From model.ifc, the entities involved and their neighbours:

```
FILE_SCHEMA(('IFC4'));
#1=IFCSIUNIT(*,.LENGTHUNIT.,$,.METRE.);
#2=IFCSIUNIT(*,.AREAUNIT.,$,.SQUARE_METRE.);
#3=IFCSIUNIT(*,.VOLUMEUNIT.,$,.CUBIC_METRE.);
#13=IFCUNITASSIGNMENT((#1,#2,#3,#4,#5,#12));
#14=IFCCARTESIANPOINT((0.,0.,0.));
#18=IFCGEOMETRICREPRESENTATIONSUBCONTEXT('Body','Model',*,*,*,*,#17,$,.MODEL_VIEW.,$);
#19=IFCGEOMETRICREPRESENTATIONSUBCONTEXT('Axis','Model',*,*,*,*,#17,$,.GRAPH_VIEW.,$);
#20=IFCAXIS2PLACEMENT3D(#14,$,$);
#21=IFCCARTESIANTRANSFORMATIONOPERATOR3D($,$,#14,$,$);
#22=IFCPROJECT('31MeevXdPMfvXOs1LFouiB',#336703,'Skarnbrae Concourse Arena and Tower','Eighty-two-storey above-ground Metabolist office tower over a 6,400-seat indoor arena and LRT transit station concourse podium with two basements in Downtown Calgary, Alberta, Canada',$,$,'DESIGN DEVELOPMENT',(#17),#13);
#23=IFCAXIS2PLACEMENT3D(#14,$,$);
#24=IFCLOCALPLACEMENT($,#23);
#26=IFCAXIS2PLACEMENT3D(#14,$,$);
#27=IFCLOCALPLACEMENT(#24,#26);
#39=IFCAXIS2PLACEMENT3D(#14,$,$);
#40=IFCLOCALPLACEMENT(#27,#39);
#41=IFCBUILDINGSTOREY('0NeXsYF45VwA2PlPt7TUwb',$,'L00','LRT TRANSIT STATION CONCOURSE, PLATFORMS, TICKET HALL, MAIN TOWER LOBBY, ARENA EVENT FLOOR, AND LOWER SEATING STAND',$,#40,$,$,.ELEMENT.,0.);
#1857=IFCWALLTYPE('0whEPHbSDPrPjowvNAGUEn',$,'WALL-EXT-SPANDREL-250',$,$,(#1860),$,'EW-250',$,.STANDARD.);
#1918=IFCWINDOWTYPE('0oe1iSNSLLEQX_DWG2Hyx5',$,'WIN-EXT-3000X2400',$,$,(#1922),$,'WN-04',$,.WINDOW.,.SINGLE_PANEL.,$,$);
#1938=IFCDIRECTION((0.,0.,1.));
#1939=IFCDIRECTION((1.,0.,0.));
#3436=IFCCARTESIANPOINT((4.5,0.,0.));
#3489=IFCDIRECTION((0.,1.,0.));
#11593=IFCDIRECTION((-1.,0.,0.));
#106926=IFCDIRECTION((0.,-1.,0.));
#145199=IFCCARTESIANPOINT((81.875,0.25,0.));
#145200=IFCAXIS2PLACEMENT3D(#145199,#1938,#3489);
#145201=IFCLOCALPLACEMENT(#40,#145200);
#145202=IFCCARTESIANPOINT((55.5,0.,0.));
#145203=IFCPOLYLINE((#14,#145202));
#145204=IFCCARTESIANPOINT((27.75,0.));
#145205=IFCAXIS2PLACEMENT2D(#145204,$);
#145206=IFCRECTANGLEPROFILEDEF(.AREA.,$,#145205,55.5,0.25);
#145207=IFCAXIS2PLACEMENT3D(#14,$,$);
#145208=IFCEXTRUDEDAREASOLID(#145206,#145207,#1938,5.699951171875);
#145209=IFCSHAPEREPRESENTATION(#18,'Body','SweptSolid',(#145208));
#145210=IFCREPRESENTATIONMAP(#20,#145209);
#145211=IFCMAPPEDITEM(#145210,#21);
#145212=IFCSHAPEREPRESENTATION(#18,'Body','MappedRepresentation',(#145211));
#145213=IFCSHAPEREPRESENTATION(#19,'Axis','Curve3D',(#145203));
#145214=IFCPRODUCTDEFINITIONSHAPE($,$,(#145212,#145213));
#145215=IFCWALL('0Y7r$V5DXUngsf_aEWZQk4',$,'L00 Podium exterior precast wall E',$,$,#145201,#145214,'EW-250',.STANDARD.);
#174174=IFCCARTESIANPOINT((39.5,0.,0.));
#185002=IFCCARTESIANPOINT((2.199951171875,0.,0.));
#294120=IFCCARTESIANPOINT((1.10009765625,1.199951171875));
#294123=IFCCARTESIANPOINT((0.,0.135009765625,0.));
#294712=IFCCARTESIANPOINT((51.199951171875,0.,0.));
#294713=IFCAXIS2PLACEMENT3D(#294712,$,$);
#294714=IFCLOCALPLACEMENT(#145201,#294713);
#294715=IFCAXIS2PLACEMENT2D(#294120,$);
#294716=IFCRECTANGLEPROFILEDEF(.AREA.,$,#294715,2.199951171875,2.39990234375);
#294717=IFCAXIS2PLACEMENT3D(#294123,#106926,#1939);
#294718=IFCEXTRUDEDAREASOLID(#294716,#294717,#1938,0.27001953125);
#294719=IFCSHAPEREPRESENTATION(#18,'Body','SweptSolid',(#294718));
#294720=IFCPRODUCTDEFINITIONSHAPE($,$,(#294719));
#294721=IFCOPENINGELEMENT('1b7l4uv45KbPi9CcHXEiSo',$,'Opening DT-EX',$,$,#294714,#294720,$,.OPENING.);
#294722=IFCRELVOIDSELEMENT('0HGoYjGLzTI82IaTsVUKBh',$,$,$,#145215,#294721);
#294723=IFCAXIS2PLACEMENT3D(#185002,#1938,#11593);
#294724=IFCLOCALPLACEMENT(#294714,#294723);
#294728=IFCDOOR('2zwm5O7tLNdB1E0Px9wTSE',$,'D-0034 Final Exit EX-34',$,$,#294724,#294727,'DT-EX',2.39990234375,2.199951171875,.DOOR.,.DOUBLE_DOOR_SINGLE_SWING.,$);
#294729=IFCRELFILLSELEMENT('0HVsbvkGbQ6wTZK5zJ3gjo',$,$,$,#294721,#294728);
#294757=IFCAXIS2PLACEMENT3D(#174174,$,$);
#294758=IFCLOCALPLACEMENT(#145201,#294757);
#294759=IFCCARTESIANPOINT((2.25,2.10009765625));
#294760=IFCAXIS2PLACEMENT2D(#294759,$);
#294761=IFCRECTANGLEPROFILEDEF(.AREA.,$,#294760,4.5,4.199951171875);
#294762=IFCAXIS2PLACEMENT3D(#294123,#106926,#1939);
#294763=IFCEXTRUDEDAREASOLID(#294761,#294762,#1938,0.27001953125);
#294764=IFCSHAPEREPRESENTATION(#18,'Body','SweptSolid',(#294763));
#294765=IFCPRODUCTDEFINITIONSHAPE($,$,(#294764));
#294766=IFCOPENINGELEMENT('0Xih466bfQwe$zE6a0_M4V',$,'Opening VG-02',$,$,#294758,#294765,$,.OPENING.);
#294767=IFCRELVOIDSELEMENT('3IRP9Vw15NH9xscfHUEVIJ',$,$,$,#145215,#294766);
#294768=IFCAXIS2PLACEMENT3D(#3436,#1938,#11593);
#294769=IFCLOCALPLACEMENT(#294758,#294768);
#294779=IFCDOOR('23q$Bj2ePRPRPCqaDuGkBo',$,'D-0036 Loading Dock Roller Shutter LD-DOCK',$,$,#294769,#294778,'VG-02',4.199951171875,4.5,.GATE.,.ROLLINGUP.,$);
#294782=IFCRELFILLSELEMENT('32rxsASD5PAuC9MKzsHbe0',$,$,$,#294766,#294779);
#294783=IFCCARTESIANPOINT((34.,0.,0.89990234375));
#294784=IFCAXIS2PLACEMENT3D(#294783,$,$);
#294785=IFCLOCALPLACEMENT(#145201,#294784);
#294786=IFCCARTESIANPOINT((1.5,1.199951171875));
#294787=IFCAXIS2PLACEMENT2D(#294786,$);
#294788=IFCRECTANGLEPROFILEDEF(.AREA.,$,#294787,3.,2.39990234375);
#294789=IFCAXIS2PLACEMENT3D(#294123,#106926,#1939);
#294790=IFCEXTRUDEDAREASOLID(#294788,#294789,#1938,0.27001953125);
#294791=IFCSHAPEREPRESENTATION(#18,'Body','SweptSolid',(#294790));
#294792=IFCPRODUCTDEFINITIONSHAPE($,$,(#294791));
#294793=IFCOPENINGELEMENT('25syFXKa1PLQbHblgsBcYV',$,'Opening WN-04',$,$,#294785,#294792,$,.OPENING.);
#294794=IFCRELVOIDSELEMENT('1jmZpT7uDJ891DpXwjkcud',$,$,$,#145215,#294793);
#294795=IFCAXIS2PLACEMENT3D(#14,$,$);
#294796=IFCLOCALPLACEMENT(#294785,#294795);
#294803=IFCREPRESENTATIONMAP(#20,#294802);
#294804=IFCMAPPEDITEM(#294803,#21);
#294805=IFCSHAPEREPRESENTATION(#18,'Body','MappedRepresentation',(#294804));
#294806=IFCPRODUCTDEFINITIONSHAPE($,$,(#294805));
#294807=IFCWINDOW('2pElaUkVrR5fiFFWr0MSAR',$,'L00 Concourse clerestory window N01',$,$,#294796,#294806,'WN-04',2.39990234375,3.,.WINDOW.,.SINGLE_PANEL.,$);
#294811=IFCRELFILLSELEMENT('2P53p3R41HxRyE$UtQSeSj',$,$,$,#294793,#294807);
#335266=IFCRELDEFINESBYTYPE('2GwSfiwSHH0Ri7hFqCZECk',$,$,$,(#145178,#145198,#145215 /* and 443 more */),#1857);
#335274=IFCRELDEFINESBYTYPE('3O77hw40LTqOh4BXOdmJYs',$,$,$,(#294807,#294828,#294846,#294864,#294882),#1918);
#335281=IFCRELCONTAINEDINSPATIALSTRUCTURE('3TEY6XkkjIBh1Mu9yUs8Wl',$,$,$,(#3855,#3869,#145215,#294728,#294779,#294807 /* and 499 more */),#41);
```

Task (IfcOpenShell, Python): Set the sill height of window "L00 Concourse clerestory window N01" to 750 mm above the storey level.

```python
import numpy as np
import ifcopenshell
import ifcopenshell.api.geometry
import ifcopenshell.geom
import ifcopenshell.util.element
import ifcopenshell.util.placement
import ifcopenshell.util.shape
import ifcopenshell.util.unit

model = ifcopenshell.open("model.ifc")
unit_scale = ifcopenshell.util.unit.calculate_unit_scale(model)

window = model.by_guid("2pElaUkVrR5fiFFWr0MSAR")
opening = window.FillsVoids[0].RelatingOpeningElement
storey = ifcopenshell.util.element.get_container(window, ifc_class="IfcBuildingStorey")
level = ifcopenshell.util.placement.get_local_placement(storey.ObjectPlacement)[2, 3]

# The opening's origin need not be at the sill, so measure its lowest point.
shape = ifcopenshell.geom.create_shape(ifcopenshell.geom.settings(), opening)
bottom = ifcopenshell.util.shape.get_shape_bottom_elevation(shape, shape.geometry) / unit_scale
dz = level + 0.75 - bottom

shift = np.array([0.0, 0.0, dz])
# The window is placed relative to its opening, so it follows when the opening moves.
matrix = ifcopenshell.util.placement.get_local_placement(opening.ObjectPlacement)
matrix[:3, 3] += shift
ifcopenshell.api.geometry.edit_object_placement(
    model, product=opening, matrix=matrix, is_si=False, should_transform_children=True
)

print(f"moved by {dz * unit_scale:+.3f} m")

model.write("model_updated.ifc")
```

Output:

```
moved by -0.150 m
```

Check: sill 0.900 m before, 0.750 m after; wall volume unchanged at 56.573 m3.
